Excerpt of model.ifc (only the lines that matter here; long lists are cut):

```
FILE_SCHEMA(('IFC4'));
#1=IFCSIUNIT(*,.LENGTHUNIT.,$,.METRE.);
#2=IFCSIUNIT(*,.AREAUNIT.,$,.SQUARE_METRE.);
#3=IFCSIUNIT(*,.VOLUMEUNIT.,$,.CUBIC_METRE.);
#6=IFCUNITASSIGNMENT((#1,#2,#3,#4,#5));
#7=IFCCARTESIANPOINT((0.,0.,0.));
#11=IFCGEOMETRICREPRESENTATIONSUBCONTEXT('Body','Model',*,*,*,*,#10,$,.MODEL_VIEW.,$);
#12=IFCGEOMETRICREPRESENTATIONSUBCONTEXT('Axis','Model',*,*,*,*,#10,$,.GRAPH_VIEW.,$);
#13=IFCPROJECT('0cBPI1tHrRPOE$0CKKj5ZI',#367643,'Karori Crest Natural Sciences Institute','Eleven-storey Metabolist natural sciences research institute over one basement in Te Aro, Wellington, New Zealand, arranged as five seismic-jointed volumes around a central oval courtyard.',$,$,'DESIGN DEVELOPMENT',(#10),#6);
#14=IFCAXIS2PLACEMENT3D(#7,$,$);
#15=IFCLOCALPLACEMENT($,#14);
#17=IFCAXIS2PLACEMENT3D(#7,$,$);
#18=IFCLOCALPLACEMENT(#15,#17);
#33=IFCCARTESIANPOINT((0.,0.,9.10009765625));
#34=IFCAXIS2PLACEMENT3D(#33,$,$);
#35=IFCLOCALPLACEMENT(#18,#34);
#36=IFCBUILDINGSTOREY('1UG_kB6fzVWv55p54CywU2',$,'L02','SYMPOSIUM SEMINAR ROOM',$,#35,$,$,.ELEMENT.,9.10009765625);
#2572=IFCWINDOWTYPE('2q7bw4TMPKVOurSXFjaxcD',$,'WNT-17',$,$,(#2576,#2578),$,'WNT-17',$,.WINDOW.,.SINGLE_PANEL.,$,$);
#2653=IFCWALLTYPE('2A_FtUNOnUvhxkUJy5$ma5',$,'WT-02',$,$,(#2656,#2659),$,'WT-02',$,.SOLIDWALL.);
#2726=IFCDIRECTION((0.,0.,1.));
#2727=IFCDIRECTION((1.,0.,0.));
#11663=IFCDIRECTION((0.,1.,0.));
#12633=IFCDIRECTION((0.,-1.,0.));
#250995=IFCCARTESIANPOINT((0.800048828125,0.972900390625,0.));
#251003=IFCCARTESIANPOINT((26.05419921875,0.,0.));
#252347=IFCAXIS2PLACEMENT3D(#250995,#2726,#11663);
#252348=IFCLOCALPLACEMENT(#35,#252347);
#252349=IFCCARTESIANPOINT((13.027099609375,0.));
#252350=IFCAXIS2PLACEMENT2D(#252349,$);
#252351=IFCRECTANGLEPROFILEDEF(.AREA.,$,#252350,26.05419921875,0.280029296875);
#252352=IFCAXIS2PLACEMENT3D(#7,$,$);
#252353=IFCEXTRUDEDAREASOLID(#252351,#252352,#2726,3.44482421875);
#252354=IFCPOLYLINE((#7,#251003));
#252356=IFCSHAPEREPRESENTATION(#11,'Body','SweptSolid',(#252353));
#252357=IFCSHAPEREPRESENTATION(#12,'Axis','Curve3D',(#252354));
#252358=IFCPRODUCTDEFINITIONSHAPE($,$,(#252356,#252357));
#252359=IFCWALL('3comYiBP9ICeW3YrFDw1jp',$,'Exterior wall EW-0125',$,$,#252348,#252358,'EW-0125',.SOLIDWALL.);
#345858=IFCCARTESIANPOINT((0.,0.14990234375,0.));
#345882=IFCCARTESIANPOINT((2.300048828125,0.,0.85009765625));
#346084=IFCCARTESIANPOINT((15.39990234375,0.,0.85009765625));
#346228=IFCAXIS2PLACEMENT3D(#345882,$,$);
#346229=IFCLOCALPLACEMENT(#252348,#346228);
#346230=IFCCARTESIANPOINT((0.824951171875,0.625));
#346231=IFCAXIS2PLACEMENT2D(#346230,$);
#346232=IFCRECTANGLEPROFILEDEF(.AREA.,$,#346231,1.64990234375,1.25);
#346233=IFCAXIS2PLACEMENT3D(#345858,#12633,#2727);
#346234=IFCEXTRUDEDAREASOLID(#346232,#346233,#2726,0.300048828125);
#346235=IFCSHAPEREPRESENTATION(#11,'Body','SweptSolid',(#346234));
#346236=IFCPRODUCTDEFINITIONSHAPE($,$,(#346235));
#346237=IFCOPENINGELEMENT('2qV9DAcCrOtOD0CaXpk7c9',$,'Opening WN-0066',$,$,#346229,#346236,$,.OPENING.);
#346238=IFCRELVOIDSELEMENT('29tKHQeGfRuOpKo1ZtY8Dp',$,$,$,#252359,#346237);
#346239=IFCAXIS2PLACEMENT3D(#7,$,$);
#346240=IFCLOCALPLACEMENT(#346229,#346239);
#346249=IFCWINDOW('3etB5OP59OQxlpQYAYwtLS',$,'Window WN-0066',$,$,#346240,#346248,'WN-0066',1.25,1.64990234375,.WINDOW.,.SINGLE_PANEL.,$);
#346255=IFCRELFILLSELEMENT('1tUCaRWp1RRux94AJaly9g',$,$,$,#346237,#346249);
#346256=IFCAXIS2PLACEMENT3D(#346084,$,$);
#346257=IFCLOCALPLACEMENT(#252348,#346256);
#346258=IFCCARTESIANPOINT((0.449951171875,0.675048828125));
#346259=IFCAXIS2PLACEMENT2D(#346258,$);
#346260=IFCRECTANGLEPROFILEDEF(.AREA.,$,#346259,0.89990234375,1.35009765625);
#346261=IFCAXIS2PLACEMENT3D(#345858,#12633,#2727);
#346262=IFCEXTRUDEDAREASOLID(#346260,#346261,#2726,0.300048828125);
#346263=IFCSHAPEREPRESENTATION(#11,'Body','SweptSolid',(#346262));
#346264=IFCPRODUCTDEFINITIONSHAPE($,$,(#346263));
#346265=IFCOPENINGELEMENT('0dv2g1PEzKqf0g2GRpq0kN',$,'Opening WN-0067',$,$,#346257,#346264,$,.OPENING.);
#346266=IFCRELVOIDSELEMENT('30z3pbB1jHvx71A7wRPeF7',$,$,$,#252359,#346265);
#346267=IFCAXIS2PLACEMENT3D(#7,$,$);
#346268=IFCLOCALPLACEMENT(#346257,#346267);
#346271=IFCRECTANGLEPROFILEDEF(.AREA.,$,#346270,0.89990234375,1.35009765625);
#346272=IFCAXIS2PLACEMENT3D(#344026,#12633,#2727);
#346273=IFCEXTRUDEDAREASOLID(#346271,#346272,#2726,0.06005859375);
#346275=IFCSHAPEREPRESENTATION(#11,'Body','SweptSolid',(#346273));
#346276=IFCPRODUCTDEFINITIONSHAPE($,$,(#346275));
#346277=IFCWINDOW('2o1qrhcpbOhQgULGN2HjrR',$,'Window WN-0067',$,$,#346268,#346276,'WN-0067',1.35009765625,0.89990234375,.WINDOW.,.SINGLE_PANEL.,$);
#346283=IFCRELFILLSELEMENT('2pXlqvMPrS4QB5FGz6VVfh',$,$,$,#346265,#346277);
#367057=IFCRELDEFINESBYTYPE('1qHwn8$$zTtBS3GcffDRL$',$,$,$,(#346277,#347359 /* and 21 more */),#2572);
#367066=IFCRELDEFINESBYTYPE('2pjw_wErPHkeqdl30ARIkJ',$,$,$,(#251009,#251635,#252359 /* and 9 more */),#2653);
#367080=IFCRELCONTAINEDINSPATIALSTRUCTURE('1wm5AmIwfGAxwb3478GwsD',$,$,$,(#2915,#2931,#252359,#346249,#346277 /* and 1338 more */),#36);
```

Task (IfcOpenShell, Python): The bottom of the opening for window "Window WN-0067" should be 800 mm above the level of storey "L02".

```python
import numpy as np
import ifcopenshell
import ifcopenshell.api.geometry
import ifcopenshell.geom
import ifcopenshell.util.element
import ifcopenshell.util.placement
import ifcopenshell.util.shape
import ifcopenshell.util.unit

model = ifcopenshell.open("model.ifc")
unit_scale = ifcopenshell.util.unit.calculate_unit_scale(model)

window = model.by_guid("2o1qrhcpbOhQgULGN2HjrR")
opening = window.FillsVoids[0].RelatingOpeningElement
storey = ifcopenshell.util.element.get_container(window, ifc_class="IfcBuildingStorey")
level = ifcopenshell.util.placement.get_local_placement(storey.ObjectPlacement)[2, 3]

# The opening's origin need not be at the sill, so measure its lowest point.
shape = ifcopenshell.geom.create_shape(ifcopenshell.geom.settings(), opening)
bottom = ifcopenshell.util.shape.get_shape_bottom_elevation(shape, shape.geometry) / unit_scale
dz = level + 0.8 / unit_scale - bottom

shift = np.array([0.0, 0.0, dz])
# The window is placed relative to its opening, so it follows when the opening moves.
matrix = ifcopenshell.util.placement.get_local_placement(opening.ObjectPlacement)
matrix[:3, 3] += shift
ifcopenshell.api.geometry.edit_object_placement(
    model, product=opening, matrix=matrix, is_si=False, should_transform_children=True
)

print(f"moved by {dz * unit_scale:+.3f} m")

model.write("model_edited.ifc")
```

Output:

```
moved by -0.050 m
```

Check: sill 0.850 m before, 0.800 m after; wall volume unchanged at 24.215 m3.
